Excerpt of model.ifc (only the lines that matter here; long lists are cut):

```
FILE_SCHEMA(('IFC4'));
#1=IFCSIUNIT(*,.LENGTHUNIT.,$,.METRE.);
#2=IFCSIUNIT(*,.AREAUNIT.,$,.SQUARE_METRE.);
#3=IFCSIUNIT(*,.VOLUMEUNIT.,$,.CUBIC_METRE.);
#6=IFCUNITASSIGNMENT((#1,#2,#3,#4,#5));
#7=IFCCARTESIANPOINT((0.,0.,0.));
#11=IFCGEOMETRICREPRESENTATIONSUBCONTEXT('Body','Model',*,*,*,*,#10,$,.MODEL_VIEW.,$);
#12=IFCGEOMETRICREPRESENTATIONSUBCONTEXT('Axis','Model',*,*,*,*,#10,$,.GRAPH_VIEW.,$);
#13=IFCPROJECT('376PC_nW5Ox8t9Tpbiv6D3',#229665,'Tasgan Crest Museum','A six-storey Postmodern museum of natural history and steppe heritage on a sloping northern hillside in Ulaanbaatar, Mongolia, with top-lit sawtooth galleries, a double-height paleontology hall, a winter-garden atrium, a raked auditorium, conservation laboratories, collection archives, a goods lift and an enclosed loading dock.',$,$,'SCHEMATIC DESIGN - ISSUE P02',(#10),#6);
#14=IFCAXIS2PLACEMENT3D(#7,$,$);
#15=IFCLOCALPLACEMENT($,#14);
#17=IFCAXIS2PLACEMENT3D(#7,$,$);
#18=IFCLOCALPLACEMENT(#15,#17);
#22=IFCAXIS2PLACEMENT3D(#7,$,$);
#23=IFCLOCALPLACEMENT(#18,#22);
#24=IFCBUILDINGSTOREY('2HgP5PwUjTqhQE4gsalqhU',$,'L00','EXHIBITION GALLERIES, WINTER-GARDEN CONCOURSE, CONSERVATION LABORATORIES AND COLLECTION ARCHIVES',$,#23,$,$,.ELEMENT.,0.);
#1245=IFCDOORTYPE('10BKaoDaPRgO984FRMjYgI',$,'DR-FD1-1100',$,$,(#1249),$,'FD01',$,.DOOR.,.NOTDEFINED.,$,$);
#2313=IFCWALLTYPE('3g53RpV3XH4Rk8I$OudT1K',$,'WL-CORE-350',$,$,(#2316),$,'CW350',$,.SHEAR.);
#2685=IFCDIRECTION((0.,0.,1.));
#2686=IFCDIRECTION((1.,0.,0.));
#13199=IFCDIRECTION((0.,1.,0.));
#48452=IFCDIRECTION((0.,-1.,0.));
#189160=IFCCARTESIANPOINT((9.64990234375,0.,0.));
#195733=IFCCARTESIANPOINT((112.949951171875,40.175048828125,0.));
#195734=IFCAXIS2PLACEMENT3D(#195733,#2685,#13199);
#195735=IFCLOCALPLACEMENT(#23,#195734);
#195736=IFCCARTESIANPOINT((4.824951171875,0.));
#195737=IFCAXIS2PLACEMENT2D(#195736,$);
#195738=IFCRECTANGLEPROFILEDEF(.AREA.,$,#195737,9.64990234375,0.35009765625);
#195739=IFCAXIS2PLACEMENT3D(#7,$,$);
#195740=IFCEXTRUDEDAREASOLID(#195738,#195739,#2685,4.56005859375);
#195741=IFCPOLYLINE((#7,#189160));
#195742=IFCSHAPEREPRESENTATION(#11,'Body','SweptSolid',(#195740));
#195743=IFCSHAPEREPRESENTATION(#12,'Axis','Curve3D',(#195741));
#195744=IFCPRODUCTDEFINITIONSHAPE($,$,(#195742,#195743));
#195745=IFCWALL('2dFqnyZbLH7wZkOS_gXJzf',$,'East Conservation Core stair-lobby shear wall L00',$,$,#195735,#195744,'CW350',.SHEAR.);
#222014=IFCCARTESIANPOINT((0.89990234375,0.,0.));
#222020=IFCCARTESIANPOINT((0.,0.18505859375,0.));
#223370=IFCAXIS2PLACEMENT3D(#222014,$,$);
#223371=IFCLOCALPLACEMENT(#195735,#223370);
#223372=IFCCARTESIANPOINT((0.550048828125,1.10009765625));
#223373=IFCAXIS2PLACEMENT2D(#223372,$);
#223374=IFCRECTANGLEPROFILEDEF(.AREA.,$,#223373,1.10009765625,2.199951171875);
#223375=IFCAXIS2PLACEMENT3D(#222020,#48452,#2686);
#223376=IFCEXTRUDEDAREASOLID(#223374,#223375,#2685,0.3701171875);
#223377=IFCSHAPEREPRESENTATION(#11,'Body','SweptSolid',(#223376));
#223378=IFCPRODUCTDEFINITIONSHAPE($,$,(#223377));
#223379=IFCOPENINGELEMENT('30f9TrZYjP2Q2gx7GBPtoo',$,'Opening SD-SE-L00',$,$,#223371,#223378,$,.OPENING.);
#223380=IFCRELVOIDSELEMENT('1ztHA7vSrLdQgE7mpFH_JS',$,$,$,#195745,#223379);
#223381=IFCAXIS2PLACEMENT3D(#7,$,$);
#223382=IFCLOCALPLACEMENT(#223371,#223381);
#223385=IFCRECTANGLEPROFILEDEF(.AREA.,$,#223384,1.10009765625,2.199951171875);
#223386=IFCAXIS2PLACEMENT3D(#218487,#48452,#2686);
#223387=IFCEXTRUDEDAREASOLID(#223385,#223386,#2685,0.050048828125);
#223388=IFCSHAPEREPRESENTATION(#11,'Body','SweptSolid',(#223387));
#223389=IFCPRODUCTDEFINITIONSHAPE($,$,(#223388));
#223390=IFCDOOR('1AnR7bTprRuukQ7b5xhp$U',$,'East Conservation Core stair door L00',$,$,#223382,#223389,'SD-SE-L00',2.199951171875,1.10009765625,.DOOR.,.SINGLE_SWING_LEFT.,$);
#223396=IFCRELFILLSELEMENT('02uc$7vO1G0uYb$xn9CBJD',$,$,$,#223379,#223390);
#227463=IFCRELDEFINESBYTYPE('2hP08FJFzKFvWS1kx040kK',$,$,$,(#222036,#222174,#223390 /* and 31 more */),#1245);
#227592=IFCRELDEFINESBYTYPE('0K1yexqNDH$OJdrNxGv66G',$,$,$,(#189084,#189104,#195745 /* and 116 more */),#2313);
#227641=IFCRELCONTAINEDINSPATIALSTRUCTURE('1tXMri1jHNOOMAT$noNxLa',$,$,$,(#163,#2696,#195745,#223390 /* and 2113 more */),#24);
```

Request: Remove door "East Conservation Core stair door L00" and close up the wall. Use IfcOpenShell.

```python
import ifcopenshell
import ifcopenshell.api.feature
import ifcopenshell.api.root
import ifcopenshell.geom
import ifcopenshell.util.shape

model = ifcopenshell.open("model.ifc")
settings = ifcopenshell.geom.settings()


def volume(element):
    """Net volume in cubic metres, openings subtracted."""
    shape = ifcopenshell.geom.create_shape(settings, element)
    return ifcopenshell.util.shape.get_volume(shape.geometry)


door = model.by_guid("1AnR7bTprRuukQ7b5xhp$U")
opening = door.FillsVoids[0].RelatingOpeningElement
wall = opening.VoidsElements[0].RelatingBuildingElement
before = volume(wall)

ifcopenshell.api.root.remove_product(model, product=door)
ifcopenshell.api.feature.remove_feature(model, feature=opening)

after = volume(wall)

print(f"wall volume {before:.3f} -> {after:.3f} m3")

model.write("model_v2.ifc")
```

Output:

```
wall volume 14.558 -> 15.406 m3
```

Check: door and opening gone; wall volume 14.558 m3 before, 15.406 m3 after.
